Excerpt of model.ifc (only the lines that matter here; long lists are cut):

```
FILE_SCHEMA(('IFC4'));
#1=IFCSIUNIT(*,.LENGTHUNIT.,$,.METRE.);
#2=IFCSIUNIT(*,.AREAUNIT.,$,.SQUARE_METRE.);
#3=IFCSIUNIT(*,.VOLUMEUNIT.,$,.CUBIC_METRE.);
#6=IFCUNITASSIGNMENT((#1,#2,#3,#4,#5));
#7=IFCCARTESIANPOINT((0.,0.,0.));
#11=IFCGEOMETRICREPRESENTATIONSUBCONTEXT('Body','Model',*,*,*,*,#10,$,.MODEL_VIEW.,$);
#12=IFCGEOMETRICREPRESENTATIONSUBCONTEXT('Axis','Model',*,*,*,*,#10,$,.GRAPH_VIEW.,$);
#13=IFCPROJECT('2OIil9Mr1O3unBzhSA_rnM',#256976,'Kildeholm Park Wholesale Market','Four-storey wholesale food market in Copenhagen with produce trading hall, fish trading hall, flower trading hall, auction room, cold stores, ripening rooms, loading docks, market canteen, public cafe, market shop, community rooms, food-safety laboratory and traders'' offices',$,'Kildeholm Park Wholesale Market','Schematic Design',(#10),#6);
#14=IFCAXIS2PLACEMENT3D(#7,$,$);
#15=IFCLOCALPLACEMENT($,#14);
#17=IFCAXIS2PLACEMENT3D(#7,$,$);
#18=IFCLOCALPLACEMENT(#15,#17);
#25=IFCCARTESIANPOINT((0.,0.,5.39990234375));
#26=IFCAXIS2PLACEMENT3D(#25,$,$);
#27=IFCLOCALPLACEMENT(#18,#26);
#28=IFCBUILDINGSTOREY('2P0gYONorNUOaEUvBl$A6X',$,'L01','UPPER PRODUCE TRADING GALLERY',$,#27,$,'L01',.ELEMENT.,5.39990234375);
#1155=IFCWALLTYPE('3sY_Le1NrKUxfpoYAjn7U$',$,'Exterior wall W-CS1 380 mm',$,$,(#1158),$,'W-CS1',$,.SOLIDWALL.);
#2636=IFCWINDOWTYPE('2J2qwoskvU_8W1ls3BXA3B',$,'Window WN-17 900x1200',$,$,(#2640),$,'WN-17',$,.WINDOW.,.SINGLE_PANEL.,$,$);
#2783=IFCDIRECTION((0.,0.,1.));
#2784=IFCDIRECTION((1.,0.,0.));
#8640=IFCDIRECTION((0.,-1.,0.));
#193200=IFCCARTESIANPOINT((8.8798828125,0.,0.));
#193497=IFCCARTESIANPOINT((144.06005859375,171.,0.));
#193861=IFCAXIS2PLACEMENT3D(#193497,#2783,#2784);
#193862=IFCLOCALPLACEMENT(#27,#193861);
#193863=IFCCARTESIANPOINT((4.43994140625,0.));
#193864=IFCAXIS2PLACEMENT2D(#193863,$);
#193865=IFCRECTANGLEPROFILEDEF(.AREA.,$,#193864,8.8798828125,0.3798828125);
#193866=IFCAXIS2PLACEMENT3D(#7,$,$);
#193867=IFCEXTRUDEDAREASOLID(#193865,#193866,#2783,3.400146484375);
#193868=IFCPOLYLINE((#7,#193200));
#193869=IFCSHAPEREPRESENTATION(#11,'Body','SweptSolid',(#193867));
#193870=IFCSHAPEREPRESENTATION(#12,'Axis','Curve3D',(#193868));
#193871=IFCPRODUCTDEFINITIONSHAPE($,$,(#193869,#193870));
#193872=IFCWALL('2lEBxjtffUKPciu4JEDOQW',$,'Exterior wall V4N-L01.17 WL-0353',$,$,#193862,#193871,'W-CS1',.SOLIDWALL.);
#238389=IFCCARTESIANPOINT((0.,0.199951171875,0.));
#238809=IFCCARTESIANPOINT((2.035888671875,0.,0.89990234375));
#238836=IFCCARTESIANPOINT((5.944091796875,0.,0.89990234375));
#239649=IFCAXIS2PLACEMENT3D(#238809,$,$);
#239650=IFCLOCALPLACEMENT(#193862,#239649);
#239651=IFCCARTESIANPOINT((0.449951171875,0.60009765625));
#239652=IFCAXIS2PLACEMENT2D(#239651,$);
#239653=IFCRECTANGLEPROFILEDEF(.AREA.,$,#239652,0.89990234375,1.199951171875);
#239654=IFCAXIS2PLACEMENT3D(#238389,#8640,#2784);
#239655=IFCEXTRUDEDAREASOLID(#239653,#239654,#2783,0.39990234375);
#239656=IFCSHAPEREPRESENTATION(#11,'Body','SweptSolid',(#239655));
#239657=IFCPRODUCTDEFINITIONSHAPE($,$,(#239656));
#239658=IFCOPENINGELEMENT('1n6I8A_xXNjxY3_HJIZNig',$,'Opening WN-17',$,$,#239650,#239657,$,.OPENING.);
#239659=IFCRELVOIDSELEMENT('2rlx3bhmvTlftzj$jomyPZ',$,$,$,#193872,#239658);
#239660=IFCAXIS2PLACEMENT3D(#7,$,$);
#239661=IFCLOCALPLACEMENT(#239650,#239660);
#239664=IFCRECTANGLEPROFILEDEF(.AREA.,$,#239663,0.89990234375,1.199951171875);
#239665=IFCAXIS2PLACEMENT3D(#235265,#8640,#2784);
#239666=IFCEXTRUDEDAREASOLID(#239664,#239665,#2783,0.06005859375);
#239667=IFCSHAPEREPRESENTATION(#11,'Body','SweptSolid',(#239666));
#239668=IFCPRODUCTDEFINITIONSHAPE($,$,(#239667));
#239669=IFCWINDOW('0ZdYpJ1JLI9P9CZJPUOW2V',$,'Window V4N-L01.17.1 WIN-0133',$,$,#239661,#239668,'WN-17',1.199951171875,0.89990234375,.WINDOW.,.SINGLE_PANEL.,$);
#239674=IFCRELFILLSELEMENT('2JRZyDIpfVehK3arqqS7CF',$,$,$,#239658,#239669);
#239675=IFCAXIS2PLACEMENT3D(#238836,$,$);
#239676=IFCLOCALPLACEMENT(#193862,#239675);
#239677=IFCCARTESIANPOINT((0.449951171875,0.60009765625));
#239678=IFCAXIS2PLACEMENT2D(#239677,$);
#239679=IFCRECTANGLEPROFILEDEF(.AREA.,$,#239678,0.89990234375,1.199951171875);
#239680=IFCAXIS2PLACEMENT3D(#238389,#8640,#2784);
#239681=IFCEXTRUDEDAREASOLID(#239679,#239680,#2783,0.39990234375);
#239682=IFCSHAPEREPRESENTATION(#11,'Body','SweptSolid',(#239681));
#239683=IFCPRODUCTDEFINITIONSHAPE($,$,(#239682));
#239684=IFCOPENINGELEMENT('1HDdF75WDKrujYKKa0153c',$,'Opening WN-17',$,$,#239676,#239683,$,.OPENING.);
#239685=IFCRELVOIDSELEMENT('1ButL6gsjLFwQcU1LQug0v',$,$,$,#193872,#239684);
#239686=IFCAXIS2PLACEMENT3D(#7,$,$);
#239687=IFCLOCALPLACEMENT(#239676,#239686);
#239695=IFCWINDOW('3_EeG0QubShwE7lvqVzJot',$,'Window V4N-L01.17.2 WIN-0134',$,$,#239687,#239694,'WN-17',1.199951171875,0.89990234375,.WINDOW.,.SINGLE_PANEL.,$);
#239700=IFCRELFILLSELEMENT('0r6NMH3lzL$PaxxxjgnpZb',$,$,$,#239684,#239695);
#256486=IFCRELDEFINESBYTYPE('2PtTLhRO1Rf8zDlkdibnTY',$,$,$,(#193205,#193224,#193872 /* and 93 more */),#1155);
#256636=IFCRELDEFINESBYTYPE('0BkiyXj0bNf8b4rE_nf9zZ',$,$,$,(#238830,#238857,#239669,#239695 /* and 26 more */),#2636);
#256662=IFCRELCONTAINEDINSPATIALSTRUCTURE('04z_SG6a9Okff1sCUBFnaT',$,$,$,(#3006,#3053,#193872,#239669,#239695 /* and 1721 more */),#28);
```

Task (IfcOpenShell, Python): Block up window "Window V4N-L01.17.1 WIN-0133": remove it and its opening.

```python
import ifcopenshell
import ifcopenshell.api.feature
import ifcopenshell.api.root
import ifcopenshell.geom
import ifcopenshell.util.shape

model = ifcopenshell.open("model.ifc")
settings = ifcopenshell.geom.settings()


def volume(element):
    """Net volume in cubic metres, openings subtracted."""
    shape = ifcopenshell.geom.create_shape(settings, element)
    return ifcopenshell.util.shape.get_volume(shape.geometry)


window = model.by_guid("0ZdYpJ1JLI9P9CZJPUOW2V")
opening = window.FillsVoids[0].RelatingOpeningElement
wall = opening.VoidsElements[0].RelatingBuildingElement
before = volume(wall)

ifcopenshell.api.root.remove_product(model, product=window)
ifcopenshell.api.feature.remove_feature(model, feature=opening)

after = volume(wall)

print(f"wall volume {before:.3f} -> {after:.3f} m3")

model.write("model-out.ifc")
```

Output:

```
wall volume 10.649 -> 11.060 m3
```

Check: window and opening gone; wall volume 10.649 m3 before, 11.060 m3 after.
